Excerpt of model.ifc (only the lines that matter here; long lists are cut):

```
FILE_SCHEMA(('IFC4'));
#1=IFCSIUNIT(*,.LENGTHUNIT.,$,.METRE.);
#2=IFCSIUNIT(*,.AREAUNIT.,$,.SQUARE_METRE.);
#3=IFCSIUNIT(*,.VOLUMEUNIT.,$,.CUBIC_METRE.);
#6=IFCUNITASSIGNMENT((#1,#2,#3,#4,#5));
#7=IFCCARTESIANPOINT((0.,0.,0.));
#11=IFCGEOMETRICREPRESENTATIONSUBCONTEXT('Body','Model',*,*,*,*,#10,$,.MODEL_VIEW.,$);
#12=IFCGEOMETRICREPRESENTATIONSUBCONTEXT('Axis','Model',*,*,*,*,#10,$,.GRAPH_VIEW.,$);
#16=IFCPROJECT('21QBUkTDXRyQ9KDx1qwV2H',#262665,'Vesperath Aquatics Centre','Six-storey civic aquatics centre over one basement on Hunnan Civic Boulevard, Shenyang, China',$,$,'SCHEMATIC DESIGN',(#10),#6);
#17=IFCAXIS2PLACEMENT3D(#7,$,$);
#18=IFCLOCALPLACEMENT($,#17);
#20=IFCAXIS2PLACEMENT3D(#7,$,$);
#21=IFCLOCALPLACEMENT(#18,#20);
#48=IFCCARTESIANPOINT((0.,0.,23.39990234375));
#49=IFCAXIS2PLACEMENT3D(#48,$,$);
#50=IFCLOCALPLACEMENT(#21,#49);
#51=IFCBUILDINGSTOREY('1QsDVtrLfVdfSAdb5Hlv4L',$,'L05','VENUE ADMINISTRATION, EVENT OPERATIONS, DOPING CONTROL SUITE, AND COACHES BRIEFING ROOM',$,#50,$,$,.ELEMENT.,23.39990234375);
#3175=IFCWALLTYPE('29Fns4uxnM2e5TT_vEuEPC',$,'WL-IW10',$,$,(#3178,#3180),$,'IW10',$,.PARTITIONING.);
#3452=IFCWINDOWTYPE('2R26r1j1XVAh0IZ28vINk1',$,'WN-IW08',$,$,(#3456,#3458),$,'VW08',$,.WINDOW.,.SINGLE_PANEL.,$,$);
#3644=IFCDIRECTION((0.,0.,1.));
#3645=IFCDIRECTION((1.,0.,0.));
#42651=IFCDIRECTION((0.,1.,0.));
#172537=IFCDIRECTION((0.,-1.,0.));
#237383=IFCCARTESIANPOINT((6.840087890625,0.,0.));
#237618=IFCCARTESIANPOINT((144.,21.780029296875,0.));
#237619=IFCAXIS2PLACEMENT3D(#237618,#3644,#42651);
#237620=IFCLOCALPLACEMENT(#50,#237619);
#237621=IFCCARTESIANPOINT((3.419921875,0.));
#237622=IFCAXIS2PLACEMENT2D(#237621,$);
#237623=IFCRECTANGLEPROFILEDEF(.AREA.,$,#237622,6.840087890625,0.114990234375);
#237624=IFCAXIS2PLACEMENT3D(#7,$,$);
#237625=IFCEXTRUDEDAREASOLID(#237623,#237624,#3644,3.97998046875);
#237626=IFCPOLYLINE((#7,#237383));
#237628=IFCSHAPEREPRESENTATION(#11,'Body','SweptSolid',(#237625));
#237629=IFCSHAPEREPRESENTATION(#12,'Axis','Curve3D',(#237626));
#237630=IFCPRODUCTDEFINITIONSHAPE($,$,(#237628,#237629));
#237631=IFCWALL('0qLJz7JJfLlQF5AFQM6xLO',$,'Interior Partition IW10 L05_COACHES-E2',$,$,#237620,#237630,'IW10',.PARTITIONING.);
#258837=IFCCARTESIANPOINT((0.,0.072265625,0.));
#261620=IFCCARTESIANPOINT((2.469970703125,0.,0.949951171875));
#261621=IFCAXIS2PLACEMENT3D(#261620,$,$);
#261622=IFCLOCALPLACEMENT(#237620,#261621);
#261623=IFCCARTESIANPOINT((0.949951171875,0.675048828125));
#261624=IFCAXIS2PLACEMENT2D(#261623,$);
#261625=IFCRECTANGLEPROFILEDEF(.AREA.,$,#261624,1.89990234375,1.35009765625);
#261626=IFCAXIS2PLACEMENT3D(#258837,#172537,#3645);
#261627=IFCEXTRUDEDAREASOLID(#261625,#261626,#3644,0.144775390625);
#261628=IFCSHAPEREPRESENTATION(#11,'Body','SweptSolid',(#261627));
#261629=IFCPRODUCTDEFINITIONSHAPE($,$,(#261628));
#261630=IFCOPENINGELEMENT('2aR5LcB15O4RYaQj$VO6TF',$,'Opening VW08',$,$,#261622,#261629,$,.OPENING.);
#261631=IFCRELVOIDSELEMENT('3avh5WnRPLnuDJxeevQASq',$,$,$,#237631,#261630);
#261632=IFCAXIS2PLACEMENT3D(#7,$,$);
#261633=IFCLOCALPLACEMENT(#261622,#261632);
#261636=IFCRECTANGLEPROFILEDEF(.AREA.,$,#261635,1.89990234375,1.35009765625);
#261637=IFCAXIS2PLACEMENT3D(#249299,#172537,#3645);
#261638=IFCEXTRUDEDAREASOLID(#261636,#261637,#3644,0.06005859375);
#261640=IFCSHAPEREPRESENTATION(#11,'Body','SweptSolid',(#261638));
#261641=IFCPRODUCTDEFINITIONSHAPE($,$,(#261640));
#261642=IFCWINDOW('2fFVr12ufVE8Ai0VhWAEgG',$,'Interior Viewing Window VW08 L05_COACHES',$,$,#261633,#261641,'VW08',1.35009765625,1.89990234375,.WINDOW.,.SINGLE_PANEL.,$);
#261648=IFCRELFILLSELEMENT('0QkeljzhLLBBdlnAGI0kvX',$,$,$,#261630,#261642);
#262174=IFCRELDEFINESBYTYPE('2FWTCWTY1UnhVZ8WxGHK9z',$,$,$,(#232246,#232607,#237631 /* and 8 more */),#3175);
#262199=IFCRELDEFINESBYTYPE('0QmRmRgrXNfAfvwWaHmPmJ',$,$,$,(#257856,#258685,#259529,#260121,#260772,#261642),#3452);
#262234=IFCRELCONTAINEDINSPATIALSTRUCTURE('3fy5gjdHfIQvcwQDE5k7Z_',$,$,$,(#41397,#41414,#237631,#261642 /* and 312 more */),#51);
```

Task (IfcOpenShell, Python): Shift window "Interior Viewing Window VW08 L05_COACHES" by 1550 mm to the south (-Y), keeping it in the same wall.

```python
import ifcopenshell
import ifcopenshell.api.geometry
import ifcopenshell.util.placement
import ifcopenshell.util.unit

model = ifcopenshell.open("model.ifc")
unit_scale = ifcopenshell.util.unit.calculate_unit_scale(model)

window = model.by_guid("2fFVr12ufVE8Ai0VhWAEgG")
opening = window.FillsVoids[0].RelatingOpeningElement
wall = opening.VoidsElements[0].RelatingBuildingElement

wall_matrix = ifcopenshell.util.placement.get_local_placement(wall.ObjectPlacement)
shift = wall_matrix[:3, 0] * -1.55 / unit_scale
before = ifcopenshell.util.placement.get_local_placement(window.ObjectPlacement)[:3, 3].copy()

# The window is placed relative to its opening, so it follows when the opening moves.
matrix = ifcopenshell.util.placement.get_local_placement(opening.ObjectPlacement)
matrix[:3, 3] += shift
ifcopenshell.api.geometry.edit_object_placement(
    model, product=opening, matrix=matrix, is_si=False, should_transform_children=True
)

after = ifcopenshell.util.placement.get_local_placement(window.ObjectPlacement)[:3, 3]
print("window moved by", (after - before).round(3) + 0.0)

model.write("model_rev.ifc")
```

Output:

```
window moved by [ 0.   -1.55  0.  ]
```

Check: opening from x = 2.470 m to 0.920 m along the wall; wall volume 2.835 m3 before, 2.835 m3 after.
